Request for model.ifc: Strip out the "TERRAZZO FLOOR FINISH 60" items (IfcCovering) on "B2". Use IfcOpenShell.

First a look at what the model holds.

```python
import ifcopenshell
import ifcopenshell.util.element

model = ifcopenshell.open("model.ifc")
print(model.schema)
storey = next(s for s in model.by_type("IfcBuildingStorey") if s.Name == "B2")
coverings = [e for e in ifcopenshell.util.element.get_decomposition(storey) if e.is_a("IfcCovering")]
seen = {}
for e in coverings:
    element_type = ifcopenshell.util.element.get_type(e)
    name = element_type.Name if element_type not in (None, e) else None
    seen[name] = seen.get(name, 0) + 1
for name, count in sorted(seen.items(), key=str):
    print(count, "x", name)
```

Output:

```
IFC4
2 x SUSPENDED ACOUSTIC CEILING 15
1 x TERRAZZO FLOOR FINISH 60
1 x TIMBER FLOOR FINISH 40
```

```python
import ifcopenshell
import ifcopenshell.api.root
import ifcopenshell.util.element

model = ifcopenshell.open("model.ifc")

storey = next(s for s in model.by_type("IfcBuildingStorey") if s.Name == "B2")
coverings = [e for e in ifcopenshell.util.element.get_decomposition(storey) if e.is_a("IfcCovering")]
targets = [e for e in coverings if (t := ifcopenshell.util.element.get_type(e)) not in (None, e) and t.Name == "TERRAZZO FLOOR FINISH 60"]

for e in targets:
    ifcopenshell.api.root.remove_product(model, product=e)
print(len(targets), "removed")

model.write("model_updated.ifc")
```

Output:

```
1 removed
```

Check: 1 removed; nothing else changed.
